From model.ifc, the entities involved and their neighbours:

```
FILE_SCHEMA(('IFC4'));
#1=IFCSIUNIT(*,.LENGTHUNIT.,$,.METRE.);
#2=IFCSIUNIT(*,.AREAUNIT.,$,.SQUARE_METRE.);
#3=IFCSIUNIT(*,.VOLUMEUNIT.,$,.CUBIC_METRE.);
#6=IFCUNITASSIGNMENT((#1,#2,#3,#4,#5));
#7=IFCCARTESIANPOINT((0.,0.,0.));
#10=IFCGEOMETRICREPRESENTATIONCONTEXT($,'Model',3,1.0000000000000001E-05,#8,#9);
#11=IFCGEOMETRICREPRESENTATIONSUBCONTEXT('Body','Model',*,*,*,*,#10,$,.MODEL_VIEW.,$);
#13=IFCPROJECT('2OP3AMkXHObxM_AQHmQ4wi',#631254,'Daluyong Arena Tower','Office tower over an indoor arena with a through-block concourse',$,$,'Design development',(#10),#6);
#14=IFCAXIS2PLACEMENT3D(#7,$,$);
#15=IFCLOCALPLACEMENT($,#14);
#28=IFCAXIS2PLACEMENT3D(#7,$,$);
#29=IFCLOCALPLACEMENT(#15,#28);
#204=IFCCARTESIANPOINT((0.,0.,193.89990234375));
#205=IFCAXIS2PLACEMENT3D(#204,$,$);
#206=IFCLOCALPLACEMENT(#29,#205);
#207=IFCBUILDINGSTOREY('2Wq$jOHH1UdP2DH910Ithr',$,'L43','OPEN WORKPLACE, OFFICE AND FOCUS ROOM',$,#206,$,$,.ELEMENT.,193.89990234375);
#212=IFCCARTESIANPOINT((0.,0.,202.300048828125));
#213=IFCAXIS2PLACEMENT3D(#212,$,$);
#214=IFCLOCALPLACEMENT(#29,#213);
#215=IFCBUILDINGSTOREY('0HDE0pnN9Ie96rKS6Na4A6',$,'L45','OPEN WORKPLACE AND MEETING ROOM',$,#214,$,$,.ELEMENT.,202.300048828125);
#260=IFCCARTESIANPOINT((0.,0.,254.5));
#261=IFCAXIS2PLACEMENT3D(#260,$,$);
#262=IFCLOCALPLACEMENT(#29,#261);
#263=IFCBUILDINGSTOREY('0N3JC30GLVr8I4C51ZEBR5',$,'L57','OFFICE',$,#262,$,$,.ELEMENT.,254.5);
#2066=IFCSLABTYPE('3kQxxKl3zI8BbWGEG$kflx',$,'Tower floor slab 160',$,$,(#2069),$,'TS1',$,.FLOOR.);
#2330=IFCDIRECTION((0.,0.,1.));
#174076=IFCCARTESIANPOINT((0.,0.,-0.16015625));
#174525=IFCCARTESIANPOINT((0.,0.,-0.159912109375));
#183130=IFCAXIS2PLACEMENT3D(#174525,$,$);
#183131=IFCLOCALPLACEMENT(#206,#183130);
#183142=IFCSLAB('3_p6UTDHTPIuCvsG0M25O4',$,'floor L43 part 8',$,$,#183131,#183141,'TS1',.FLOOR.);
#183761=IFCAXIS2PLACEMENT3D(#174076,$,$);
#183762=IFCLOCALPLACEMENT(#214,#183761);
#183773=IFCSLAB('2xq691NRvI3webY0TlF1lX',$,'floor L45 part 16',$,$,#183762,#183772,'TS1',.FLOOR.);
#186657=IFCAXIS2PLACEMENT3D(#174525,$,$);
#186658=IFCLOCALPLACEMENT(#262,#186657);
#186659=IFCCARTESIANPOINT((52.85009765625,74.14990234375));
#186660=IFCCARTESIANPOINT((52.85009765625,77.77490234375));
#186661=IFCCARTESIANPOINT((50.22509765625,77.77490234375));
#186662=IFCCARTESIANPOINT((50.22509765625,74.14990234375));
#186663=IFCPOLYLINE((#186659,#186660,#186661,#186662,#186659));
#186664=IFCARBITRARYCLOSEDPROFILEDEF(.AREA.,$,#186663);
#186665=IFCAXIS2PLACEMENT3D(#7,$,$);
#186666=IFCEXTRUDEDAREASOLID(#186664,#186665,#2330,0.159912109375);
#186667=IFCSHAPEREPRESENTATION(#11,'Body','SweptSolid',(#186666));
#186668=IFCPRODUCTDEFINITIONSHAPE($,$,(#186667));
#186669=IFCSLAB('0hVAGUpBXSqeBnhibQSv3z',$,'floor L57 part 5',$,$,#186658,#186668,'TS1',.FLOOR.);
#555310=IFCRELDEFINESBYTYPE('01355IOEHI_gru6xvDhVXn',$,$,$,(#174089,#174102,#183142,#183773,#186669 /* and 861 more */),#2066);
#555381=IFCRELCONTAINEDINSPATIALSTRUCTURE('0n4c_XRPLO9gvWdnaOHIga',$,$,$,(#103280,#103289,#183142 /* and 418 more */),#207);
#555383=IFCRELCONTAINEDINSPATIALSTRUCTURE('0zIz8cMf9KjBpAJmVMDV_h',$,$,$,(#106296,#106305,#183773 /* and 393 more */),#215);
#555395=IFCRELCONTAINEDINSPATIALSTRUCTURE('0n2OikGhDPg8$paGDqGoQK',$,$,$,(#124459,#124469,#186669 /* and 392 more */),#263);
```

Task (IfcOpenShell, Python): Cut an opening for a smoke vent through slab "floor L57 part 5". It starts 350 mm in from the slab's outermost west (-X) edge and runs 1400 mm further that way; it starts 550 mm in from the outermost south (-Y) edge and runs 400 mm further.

```python
import numpy as np
import ifcopenshell
import ifcopenshell.api.feature
import ifcopenshell.api.geometry
import ifcopenshell.api.root
import ifcopenshell.geom
import ifcopenshell.util.placement
import ifcopenshell.util.representation
import ifcopenshell.util.shape
import ifcopenshell.util.unit

model = ifcopenshell.open("model.ifc")
unit_scale = ifcopenshell.util.unit.calculate_unit_scale(model)
settings = ifcopenshell.geom.settings()


def volume(element):
    """Net volume in cubic metres, openings subtracted."""
    shape = ifcopenshell.geom.create_shape(settings, element)
    return ifcopenshell.util.shape.get_volume(shape.geometry)


slab = model.by_guid("0hVAGUpBXSqeBnhibQSv3z")
before = volume(slab)

# Extent in the slab's own axes, in metres. The edges named are its -X and -Y sides.
slab_shape = ifcopenshell.geom.create_shape(settings, slab)
vertices = ifcopenshell.util.shape.get_vertices(slab_shape.geometry)
x_min, y_min, bottom = vertices.min(axis=0)
top = vertices[:, 2].max()

opening = ifcopenshell.api.root.create_entity(model, ifc_class="IfcOpeningElement", name="Smoke vent opening", predefined_type="OPENING")
context = ifcopenshell.util.representation.get_context(model, "Model", "Body", "MODEL_VIEW")
width, depth = 1.4, 0.4
outline = [(0.0, 0.0), (width, 0.0), (width, depth), (0.0, depth), (0.0, 0.0)]
# Overshoot both faces by 50 mm so the cut is clean.
shape = ifcopenshell.api.geometry.add_slab_representation(
    model, context=context, depth=top - bottom + 0.1, polyline=outline
)
ifcopenshell.api.geometry.assign_representation(model, product=opening, representation=shape)

matrix = ifcopenshell.util.placement.get_local_placement(slab.ObjectPlacement)
matrix[:, 3] = matrix @ np.append(np.array([x_min + 0.35, y_min + 0.55, bottom - 0.05]) / unit_scale, 1.0)
ifcopenshell.api.geometry.edit_object_placement(model, product=opening, matrix=matrix, is_si=False)
ifcopenshell.api.feature.add_feature(model, feature=opening, element=slab)

after = volume(slab)

print(f"slab volume {before:.3f} -> {after:.3f} m3")

model.write("model_updated.ifc")
```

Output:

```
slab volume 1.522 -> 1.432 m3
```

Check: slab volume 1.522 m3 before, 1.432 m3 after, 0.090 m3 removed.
